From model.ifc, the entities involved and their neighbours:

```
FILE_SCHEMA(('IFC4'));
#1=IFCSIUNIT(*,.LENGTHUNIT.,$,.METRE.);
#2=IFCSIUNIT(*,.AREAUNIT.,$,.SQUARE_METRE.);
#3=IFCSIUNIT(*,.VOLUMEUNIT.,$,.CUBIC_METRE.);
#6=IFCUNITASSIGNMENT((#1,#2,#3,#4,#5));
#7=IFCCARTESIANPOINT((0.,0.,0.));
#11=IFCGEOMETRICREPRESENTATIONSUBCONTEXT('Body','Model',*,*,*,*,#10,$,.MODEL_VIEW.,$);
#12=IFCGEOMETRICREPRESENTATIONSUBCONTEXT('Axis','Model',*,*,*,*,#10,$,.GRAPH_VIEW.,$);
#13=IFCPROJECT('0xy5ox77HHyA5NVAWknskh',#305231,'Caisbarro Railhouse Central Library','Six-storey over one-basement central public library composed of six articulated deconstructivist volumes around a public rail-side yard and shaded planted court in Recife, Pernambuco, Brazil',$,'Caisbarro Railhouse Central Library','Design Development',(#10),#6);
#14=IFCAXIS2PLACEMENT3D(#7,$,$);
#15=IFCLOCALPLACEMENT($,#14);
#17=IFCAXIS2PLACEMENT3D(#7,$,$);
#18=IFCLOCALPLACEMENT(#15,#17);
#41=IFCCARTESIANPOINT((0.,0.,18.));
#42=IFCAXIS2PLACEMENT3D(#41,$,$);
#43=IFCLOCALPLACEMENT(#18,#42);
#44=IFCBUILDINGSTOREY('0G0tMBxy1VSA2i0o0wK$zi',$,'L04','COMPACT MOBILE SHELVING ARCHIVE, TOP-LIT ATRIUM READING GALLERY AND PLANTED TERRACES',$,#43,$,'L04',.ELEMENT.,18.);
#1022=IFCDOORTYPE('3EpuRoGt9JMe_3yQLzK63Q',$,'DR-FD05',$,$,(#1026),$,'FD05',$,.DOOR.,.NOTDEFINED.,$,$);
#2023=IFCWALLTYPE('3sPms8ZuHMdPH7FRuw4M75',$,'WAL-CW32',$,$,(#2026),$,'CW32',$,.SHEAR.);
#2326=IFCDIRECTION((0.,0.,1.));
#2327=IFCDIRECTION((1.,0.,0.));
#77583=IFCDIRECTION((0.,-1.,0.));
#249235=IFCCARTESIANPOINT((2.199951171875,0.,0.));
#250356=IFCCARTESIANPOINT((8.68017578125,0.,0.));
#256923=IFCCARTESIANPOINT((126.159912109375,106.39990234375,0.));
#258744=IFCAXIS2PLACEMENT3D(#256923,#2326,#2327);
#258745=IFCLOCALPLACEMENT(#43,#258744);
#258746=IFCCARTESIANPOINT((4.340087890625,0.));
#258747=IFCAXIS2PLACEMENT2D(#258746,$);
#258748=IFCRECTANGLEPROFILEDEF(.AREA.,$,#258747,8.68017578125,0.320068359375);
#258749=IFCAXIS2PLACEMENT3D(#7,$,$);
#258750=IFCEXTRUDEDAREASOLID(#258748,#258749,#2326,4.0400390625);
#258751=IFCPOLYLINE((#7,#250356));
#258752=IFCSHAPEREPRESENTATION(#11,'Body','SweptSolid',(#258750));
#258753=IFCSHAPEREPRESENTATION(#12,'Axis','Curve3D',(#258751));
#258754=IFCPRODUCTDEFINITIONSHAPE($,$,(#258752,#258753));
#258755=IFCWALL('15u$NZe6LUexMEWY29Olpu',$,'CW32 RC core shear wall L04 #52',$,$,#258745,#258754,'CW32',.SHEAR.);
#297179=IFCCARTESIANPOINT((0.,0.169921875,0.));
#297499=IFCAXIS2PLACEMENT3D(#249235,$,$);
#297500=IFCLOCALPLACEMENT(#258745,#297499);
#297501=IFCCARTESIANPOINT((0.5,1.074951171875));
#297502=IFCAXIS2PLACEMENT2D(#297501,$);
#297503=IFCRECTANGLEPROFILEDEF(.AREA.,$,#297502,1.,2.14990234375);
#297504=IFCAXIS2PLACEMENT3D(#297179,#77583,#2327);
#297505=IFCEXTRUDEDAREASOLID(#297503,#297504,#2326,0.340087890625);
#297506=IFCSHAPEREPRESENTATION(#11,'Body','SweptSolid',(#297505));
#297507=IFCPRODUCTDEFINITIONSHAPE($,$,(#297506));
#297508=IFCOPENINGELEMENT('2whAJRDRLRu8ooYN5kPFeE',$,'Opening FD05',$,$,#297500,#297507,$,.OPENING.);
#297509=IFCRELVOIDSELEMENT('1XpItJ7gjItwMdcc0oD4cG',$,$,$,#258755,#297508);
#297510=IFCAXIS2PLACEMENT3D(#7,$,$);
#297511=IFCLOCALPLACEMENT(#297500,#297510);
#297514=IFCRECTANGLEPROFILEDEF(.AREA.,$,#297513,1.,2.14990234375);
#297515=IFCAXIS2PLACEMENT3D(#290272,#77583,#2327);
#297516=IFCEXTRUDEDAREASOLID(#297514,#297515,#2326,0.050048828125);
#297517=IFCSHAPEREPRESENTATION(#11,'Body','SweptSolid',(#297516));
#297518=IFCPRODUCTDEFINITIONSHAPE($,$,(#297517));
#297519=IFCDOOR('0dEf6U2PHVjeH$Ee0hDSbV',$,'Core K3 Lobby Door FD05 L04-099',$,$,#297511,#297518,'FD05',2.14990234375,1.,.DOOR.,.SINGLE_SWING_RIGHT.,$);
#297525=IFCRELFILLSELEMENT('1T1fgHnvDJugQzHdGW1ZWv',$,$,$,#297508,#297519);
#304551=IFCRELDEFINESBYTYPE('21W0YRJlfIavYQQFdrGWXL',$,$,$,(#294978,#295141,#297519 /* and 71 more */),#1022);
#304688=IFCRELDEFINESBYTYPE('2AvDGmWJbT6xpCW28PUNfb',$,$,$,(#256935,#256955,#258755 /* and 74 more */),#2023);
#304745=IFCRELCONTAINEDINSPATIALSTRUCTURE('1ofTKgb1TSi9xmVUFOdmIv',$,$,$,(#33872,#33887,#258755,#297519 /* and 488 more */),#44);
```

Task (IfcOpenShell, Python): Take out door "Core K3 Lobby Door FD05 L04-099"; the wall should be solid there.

```python
import ifcopenshell
import ifcopenshell.api.feature
import ifcopenshell.api.root
import ifcopenshell.geom
import ifcopenshell.util.shape

model = ifcopenshell.open("model.ifc")
settings = ifcopenshell.geom.settings()


def volume(element):
    """Net volume in cubic metres, openings subtracted."""
    shape = ifcopenshell.geom.create_shape(settings, element)
    return ifcopenshell.util.shape.get_volume(shape.geometry)


door = model.by_guid("0dEf6U2PHVjeH$Ee0hDSbV")
opening = door.FillsVoids[0].RelatingOpeningElement
wall = opening.VoidsElements[0].RelatingBuildingElement
before = volume(wall)

ifcopenshell.api.root.remove_product(model, product=door)
ifcopenshell.api.feature.remove_feature(model, feature=opening)

after = volume(wall)

print(f"wall volume {before:.3f} -> {after:.3f} m3")

model.write("model-out.ifc")
```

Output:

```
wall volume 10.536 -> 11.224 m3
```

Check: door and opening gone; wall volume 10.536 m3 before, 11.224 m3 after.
